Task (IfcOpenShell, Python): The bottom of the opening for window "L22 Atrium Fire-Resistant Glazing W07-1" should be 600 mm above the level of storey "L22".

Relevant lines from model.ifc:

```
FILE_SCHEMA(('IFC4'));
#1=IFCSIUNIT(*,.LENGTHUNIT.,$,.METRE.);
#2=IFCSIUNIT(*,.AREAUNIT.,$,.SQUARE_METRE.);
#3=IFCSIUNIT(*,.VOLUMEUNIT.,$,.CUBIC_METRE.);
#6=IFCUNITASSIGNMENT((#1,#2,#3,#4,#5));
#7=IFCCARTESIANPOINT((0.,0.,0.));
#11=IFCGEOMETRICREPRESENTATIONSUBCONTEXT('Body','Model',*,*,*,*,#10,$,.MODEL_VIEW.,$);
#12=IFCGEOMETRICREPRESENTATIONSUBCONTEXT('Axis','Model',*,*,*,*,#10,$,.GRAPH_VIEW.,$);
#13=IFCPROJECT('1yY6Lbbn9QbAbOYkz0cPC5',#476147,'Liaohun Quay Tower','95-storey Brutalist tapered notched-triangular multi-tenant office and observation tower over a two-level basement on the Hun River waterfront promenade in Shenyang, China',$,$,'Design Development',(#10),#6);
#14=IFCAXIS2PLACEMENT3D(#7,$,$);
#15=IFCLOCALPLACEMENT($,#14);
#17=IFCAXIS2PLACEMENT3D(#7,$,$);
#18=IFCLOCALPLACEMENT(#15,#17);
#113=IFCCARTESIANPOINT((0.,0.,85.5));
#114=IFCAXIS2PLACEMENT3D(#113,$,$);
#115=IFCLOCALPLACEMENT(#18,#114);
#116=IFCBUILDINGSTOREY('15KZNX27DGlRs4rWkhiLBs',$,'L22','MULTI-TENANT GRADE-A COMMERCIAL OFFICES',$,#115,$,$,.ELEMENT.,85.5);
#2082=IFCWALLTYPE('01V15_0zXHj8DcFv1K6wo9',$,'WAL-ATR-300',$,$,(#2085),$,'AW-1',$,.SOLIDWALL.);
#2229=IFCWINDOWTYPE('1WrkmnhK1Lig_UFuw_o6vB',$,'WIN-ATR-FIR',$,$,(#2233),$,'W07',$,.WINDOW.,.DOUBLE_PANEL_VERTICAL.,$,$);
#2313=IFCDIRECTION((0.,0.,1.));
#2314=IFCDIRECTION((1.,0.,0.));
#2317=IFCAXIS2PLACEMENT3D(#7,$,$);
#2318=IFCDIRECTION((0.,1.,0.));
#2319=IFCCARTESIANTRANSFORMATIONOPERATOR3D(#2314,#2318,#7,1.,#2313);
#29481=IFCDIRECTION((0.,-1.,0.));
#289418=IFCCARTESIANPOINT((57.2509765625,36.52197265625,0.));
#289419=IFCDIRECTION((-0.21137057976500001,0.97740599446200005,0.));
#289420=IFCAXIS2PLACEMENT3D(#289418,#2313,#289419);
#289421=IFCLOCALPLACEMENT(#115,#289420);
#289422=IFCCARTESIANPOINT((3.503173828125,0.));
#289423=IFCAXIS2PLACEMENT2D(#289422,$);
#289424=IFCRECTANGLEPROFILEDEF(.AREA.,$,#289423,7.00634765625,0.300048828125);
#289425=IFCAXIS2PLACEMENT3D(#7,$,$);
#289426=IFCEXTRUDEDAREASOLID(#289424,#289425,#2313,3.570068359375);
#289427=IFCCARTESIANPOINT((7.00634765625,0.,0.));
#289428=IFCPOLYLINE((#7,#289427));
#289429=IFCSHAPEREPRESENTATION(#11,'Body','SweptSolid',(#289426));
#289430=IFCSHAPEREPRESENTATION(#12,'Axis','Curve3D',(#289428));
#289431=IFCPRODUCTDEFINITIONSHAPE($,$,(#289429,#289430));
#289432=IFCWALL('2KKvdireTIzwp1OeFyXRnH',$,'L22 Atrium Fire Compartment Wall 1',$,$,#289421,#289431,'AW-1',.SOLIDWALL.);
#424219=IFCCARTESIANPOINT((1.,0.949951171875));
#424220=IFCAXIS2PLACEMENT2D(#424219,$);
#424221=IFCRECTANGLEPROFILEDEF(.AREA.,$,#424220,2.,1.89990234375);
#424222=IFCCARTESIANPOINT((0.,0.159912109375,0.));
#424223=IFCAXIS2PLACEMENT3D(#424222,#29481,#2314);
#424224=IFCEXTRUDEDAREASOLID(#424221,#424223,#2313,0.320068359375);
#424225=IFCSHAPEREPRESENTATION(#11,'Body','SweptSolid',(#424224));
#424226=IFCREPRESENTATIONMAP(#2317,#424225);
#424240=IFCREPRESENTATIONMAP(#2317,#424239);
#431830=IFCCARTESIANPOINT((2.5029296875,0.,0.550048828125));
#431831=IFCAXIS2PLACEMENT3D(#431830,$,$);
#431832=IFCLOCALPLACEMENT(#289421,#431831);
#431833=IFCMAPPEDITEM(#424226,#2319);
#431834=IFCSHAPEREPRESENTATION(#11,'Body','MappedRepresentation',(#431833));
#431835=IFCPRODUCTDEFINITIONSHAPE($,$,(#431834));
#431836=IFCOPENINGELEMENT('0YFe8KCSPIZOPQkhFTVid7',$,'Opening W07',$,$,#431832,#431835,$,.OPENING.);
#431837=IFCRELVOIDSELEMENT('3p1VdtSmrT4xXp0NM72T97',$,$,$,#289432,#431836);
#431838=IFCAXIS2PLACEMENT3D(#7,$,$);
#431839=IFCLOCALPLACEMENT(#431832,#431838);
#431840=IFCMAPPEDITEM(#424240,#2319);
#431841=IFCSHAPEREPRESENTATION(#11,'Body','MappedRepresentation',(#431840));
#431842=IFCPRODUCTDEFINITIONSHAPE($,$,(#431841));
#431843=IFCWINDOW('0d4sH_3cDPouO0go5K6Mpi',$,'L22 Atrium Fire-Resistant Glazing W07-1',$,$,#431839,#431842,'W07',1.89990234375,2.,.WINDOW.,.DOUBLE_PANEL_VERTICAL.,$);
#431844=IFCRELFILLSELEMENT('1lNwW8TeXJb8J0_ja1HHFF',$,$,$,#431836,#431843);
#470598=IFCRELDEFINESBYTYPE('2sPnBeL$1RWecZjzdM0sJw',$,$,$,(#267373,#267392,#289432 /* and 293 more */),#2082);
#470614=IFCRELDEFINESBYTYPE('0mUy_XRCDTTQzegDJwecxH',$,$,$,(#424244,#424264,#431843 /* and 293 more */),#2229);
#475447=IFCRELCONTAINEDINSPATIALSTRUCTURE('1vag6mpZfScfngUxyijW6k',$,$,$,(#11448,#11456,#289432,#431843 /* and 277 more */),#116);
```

```python
import numpy as np
import ifcopenshell
import ifcopenshell.api.geometry
import ifcopenshell.geom
import ifcopenshell.util.element
import ifcopenshell.util.placement
import ifcopenshell.util.shape
import ifcopenshell.util.unit

model = ifcopenshell.open("model.ifc")
unit_scale = ifcopenshell.util.unit.calculate_unit_scale(model)

window = model.by_guid("0d4sH_3cDPouO0go5K6Mpi")
opening = window.FillsVoids[0].RelatingOpeningElement
storey = ifcopenshell.util.element.get_container(window, ifc_class="IfcBuildingStorey")
level = ifcopenshell.util.placement.get_local_placement(storey.ObjectPlacement)[2, 3]

# The opening's origin need not be at the sill, so measure its lowest point.
shape = ifcopenshell.geom.create_shape(ifcopenshell.geom.settings(), opening)
bottom = ifcopenshell.util.shape.get_shape_bottom_elevation(shape, shape.geometry) / unit_scale
dz = level + 0.6 / unit_scale - bottom

shift = np.array([0.0, 0.0, dz])
# The window is placed relative to its opening, so it follows when the opening moves.
matrix = ifcopenshell.util.placement.get_local_placement(opening.ObjectPlacement)
matrix[:3, 3] += shift
ifcopenshell.api.geometry.edit_object_placement(
    model, product=opening, matrix=matrix, is_si=False, should_transform_children=True
)

print(f"moved by {dz * unit_scale:+.3f} m")

model.write("model-out.ifc")
```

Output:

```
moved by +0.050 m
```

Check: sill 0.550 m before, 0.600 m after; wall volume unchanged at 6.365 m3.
